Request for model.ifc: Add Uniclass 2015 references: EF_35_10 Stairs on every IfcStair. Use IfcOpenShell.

First a look at what the model holds.

```python
import ifcopenshell

model = ifcopenshell.open("model.ifc")
print(model.schema)
print("classifications:", [c.Name for c in model.by_type("IfcClassification")])
for ifc_class in ("IfcDoor", "IfcRoof", "IfcStair", "IfcWall", "IfcWindow"):
    print(ifc_class, len(model.by_type(ifc_class)))
```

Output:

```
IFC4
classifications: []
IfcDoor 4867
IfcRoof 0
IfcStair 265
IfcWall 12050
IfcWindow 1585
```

```python
import ifcopenshell
import ifcopenshell.api.classification

model = ifcopenshell.open("model.ifc")

system = ifcopenshell.api.classification.add_classification(model, classification="Uniclass 2015")

codes = {
    "IfcStair": ("EF_35_10", "Stairs"),
}
for ifc_class, (code, name) in codes.items():
    products = model.by_type(ifc_class)
    ifcopenshell.api.classification.add_reference(
        model, products=products, classification=system, identification=code, name=name
    )
    print(code, len(products))

model.write("model_updated.ifc")
```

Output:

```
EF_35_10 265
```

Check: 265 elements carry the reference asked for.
